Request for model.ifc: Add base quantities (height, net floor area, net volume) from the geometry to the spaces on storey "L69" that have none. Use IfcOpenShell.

First a look at what the model holds.

```python
import ifcopenshell
import ifcopenshell.util.element
import ifcopenshell.util.unit

model = ifcopenshell.open("model.ifc")
print(model.schema)
for unit_type in ("LENGTHUNIT", "AREAUNIT", "VOLUMEUNIT"):
    print(unit_type, ifcopenshell.util.unit.calculate_unit_scale(model, unit_type))
storey = next(s for s in model.by_type("IfcBuildingStorey") if s.Name == "L69")
spaces = [e for e in ifcopenshell.util.element.get_decomposition(storey) if e.is_a("IfcSpace")]
for e in sorted(spaces, key=lambda e: e.id()):
    print(e.id(), e.is_a(), e.Name, list(ifcopenshell.util.element.get_psets(e, qtos_only=True)), sep=" | ")
```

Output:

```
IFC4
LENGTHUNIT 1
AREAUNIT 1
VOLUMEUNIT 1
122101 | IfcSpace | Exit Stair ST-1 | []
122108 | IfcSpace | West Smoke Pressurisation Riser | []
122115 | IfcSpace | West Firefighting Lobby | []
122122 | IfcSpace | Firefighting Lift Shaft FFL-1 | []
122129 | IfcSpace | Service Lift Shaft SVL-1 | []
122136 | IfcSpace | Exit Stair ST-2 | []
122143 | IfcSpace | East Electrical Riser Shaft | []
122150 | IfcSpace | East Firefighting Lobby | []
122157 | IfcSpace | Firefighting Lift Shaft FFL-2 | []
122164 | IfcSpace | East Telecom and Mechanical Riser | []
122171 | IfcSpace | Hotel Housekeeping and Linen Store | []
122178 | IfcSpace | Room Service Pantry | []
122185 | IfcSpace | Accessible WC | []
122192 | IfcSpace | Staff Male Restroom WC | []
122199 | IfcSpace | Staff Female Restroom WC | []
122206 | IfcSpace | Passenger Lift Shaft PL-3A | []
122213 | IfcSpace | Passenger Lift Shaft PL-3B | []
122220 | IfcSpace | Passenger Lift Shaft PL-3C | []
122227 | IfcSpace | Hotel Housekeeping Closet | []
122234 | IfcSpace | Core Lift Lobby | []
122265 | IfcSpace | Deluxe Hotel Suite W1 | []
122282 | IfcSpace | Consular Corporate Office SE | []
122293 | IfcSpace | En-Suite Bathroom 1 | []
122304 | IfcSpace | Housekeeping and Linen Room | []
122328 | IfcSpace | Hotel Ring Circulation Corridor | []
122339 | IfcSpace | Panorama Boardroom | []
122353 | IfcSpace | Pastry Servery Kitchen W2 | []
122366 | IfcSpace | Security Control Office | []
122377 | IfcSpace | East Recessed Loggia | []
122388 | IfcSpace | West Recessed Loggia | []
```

```python
import ifcopenshell
import ifcopenshell.api.pset
import ifcopenshell.geom
import ifcopenshell.util.element
import ifcopenshell.util.shape
import ifcopenshell.util.unit

model = ifcopenshell.open("model.ifc")
unit_scale = ifcopenshell.util.unit.calculate_unit_scale(model)
area_scale = ifcopenshell.util.unit.calculate_unit_scale(model, "AREAUNIT")
volume_scale = ifcopenshell.util.unit.calculate_unit_scale(model, "VOLUMEUNIT")
settings = ifcopenshell.geom.settings()

storey = next(s for s in model.by_type("IfcBuildingStorey") if s.Name == "L69")
spaces = [e for e in ifcopenshell.util.element.get_decomposition(storey) if e.is_a("IfcSpace")]

for e in sorted(spaces, key=lambda e: e.id()):
    if ifcopenshell.util.element.get_psets(e, qtos_only=True, should_inherit=False):
        continue
    # Geometry comes back in metres, in the element's own axes.
    shape = ifcopenshell.geom.create_shape(settings, e)
    values = {
        "Height": ifcopenshell.util.shape.get_z(shape.geometry) / unit_scale,
        "NetFloorArea": ifcopenshell.util.shape.get_footprint_area(shape.geometry) / area_scale,
        "NetVolume": ifcopenshell.util.shape.get_volume(shape.geometry) / volume_scale,
    }
    qto = ifcopenshell.api.pset.add_qto(model, product=e, name="Qto_SpaceBaseQuantities")
    ifcopenshell.api.pset.edit_qto(model, qto=qto, properties=values)
    print(e.id(), {k: round(v, 3) for k, v in values.items()})

model.write("model_edited.ifc")
```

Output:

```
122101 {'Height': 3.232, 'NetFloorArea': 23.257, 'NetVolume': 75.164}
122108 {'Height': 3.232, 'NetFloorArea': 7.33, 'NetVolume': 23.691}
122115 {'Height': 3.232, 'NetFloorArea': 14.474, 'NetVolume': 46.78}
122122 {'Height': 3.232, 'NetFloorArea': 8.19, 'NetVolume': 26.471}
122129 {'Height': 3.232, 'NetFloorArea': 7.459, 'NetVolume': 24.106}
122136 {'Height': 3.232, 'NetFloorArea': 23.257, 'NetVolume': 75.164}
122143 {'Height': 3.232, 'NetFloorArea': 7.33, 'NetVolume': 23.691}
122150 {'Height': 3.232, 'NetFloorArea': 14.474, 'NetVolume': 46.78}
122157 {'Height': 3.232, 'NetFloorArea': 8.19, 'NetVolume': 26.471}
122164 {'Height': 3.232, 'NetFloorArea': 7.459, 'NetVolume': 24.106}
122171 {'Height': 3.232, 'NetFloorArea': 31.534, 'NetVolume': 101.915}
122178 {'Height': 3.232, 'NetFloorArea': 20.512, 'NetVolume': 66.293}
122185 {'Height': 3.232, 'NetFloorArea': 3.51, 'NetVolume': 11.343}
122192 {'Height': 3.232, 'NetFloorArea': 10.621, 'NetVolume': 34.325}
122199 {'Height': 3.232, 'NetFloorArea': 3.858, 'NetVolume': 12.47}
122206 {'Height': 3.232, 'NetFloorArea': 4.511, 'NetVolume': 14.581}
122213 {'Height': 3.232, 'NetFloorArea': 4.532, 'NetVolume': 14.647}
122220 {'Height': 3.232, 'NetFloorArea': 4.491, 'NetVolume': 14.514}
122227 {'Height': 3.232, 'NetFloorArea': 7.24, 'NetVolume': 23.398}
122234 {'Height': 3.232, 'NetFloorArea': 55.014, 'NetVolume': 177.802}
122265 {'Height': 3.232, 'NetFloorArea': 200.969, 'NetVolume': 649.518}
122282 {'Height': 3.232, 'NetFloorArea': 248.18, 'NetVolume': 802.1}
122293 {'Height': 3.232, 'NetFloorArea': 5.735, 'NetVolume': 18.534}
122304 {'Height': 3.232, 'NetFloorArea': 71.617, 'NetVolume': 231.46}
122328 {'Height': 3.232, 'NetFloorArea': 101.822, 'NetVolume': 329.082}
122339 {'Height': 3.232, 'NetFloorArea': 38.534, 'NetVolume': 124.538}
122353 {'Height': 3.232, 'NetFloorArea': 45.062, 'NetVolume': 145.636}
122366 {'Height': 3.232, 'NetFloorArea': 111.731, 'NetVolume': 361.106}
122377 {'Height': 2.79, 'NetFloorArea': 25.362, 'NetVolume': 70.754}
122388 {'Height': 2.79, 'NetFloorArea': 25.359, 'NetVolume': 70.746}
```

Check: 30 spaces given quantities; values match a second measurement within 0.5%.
